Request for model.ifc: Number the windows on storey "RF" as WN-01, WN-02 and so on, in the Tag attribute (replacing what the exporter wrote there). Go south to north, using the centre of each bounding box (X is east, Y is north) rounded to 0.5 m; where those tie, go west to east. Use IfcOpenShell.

First a look at what the model holds.

```python
import ifcopenshell
import ifcopenshell.util.element
import ifcopenshell.util.placement

model = ifcopenshell.open("model.ifc")
print(model.schema)
storey = next(s for s in model.by_type("IfcBuildingStorey") if s.Name == "RF")
windows = [e for e in ifcopenshell.util.element.get_decomposition(storey) if e.is_a("IfcWindow")]
for e in sorted(windows, key=lambda e: e.id()):
    origin = ifcopenshell.util.placement.get_local_placement(e.ObjectPlacement)[:3, 3]
    print(e.id(), e.Tag, e.Name, origin.round(2) + 0.0, sep=" | ")
```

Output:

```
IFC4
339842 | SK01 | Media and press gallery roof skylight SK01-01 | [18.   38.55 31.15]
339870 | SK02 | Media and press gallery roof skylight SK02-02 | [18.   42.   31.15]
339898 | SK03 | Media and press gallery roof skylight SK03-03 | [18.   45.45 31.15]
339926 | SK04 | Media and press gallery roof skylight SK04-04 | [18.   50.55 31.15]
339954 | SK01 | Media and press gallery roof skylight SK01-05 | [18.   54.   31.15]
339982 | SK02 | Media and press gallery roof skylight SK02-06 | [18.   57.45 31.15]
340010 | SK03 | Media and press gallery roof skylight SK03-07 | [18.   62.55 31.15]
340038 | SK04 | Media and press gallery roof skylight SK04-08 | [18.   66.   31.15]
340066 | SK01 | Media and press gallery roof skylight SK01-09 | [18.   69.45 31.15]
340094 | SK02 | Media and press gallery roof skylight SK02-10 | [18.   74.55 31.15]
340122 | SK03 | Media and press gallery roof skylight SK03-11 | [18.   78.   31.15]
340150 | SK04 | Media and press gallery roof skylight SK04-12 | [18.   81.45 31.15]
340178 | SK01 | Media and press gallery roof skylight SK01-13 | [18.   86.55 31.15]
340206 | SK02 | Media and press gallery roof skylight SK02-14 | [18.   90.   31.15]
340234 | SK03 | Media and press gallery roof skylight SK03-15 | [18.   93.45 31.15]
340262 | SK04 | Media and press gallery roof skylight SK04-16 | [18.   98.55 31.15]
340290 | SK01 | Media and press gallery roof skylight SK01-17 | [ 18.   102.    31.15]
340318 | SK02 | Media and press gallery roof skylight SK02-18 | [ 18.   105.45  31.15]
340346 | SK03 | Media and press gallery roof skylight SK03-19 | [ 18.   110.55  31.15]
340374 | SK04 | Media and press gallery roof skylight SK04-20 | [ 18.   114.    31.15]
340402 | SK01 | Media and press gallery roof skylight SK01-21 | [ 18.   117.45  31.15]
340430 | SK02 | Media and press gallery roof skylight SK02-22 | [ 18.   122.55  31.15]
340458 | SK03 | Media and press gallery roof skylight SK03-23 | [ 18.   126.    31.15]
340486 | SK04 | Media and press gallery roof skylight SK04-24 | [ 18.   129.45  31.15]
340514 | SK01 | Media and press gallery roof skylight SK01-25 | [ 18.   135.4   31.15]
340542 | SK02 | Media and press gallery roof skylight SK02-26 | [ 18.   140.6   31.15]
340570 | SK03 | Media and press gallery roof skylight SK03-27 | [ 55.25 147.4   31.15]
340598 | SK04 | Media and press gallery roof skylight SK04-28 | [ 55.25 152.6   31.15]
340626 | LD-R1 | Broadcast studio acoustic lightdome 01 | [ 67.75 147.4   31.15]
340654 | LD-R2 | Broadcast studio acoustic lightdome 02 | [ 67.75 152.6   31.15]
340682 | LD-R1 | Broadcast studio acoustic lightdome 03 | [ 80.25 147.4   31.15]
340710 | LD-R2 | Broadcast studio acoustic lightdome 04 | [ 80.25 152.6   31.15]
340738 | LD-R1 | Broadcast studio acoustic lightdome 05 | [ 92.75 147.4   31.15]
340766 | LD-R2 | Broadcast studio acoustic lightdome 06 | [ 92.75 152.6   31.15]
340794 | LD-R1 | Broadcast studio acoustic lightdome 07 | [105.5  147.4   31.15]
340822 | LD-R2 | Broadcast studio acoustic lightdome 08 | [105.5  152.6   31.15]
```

```python
import ifcopenshell
import ifcopenshell.geom
import ifcopenshell.util.element
import ifcopenshell.util.shape

model = ifcopenshell.open("model.ifc")
settings = ifcopenshell.geom.settings()
settings.set("use-world-coords", True)


def centre(element):
    shape = ifcopenshell.geom.create_shape(settings, element)
    return ifcopenshell.util.shape.get_bbox_centroid(shape.geometry)


storey = next(s for s in model.by_type("IfcBuildingStorey") if s.Name == "RF")
windows = [e for e in ifcopenshell.util.element.get_decomposition(storey) if e.is_a("IfcWindow")]

# Insertion points can sit at a corner or the storey origin, so sort by the geometry (in metres).
centres = {e: centre(e) for e in windows}
windows.sort(key=lambda e: (round(centres[e][1] / 0.5), centres[e][0]))

for i, e in enumerate(windows, start=1):
    number = f"WN-{i:02d}"
    e.Tag = number
    print(e.id(), number)

model.write("model_rev.ifc")
```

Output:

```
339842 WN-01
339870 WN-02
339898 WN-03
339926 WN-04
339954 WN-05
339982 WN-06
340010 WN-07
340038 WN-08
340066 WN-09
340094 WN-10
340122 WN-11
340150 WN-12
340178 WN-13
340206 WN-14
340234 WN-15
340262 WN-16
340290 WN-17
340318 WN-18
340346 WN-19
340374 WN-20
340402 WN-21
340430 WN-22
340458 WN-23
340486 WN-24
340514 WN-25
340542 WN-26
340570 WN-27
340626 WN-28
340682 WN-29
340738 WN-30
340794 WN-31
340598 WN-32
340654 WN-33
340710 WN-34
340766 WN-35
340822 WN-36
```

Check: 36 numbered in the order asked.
